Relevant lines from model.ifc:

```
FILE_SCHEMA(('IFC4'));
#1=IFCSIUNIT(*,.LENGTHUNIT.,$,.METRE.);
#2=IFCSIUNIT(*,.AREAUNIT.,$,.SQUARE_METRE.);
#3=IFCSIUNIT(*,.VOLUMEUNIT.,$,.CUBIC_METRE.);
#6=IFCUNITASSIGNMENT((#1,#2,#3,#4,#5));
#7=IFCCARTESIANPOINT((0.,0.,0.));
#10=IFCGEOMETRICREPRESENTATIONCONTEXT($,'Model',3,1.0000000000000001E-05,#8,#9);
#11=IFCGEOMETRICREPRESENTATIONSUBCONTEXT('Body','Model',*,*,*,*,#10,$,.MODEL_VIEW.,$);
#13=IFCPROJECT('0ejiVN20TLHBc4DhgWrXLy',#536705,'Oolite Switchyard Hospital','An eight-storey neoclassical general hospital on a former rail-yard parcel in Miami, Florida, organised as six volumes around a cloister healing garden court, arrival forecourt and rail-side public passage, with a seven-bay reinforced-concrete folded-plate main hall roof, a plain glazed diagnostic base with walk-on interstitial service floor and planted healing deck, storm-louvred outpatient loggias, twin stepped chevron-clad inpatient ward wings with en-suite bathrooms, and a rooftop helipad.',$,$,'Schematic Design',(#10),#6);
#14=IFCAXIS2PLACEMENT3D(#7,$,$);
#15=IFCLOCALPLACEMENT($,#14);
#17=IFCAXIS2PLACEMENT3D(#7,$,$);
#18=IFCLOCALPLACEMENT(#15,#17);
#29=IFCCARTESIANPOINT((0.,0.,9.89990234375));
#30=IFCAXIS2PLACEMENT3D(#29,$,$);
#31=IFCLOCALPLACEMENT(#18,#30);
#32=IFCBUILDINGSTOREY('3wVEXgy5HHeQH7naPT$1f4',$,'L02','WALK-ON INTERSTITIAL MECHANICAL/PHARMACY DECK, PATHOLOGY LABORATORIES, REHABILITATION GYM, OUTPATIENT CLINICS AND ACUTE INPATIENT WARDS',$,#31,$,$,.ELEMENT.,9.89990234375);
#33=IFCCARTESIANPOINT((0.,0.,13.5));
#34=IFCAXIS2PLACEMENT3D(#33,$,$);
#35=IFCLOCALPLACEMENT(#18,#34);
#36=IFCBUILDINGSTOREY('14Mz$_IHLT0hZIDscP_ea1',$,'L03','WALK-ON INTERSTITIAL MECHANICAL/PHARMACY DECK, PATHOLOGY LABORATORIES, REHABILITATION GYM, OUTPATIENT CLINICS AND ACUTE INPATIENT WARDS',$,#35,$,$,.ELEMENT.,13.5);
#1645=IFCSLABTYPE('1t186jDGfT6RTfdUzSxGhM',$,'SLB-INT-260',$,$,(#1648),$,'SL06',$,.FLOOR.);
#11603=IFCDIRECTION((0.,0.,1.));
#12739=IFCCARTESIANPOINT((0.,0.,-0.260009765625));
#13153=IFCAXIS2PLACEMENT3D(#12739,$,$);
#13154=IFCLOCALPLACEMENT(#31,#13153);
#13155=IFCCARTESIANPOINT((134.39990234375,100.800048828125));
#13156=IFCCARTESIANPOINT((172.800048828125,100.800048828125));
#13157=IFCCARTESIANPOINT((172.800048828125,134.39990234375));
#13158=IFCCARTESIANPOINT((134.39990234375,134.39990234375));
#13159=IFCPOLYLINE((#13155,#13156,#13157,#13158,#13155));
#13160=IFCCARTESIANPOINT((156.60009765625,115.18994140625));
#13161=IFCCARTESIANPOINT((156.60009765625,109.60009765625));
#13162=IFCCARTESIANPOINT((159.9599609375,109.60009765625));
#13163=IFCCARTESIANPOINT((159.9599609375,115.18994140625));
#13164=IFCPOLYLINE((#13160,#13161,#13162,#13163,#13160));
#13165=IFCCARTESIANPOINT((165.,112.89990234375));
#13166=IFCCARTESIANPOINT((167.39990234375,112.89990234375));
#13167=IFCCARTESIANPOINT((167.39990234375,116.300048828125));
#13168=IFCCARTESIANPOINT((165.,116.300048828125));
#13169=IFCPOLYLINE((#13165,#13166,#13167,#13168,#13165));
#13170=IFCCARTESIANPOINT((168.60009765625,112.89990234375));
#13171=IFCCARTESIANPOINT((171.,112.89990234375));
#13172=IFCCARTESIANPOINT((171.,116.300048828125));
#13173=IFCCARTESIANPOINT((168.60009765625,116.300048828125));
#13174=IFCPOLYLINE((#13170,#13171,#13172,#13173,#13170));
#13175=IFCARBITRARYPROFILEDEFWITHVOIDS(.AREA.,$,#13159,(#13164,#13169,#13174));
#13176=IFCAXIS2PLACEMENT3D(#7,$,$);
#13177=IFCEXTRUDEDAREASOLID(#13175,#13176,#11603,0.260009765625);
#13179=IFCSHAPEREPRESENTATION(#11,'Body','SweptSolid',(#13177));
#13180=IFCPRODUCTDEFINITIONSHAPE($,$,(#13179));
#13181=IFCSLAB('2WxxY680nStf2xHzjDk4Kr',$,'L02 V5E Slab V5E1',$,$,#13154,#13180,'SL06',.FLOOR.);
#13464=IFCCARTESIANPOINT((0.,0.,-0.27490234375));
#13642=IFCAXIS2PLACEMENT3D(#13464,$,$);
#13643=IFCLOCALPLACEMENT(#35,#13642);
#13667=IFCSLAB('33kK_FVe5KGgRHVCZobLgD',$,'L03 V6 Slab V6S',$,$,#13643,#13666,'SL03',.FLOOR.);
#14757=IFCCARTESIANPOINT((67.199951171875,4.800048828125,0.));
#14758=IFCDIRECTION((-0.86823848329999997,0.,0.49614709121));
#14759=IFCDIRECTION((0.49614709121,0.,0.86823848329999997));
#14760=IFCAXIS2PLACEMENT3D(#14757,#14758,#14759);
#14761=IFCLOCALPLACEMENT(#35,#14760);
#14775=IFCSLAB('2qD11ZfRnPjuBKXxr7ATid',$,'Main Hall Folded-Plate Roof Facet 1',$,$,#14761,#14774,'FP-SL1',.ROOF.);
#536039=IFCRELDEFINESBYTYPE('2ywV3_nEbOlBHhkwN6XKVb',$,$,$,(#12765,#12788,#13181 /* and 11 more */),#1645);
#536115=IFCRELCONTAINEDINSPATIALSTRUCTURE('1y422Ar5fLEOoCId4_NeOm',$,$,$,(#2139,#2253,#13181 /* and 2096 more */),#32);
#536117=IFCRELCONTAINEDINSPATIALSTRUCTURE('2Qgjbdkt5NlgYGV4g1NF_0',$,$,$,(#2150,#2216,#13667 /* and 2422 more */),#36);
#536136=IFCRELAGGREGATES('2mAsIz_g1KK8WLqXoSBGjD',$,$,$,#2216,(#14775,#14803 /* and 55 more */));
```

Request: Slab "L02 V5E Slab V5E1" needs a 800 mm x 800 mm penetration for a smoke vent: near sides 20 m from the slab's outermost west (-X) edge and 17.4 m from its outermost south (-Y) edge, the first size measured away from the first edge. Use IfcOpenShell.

```python
import numpy as np
import ifcopenshell
import ifcopenshell.api.feature
import ifcopenshell.api.geometry
import ifcopenshell.api.root
import ifcopenshell.geom
import ifcopenshell.util.placement
import ifcopenshell.util.representation
import ifcopenshell.util.shape
import ifcopenshell.util.unit

model = ifcopenshell.open("model.ifc")
unit_scale = ifcopenshell.util.unit.calculate_unit_scale(model)
settings = ifcopenshell.geom.settings()


def volume(element):
    """Net volume in cubic metres, openings subtracted."""
    shape = ifcopenshell.geom.create_shape(settings, element)
    return ifcopenshell.util.shape.get_volume(shape.geometry)


slab = model.by_guid("2WxxY680nStf2xHzjDk4Kr")
before = volume(slab)

# Extent in the slab's own axes, in metres. The edges named are its -X and -Y sides.
slab_shape = ifcopenshell.geom.create_shape(settings, slab)
vertices = ifcopenshell.util.shape.get_vertices(slab_shape.geometry)
x_min, y_min, bottom = vertices.min(axis=0)
top = vertices[:, 2].max()

opening = ifcopenshell.api.root.create_entity(model, ifc_class="IfcOpeningElement", name="Smoke vent opening", predefined_type="OPENING")
context = ifcopenshell.util.representation.get_context(model, "Model", "Body", "MODEL_VIEW")
width, depth = 0.8, 0.8
outline = [(0.0, 0.0), (width, 0.0), (width, depth), (0.0, depth), (0.0, 0.0)]
# Overshoot both faces by 50 mm so the cut is clean.
shape = ifcopenshell.api.geometry.add_slab_representation(
    model, context=context, depth=top - bottom + 0.1, polyline=outline
)
ifcopenshell.api.geometry.assign_representation(model, product=opening, representation=shape)

matrix = ifcopenshell.util.placement.get_local_placement(slab.ObjectPlacement)
matrix[:, 3] = matrix @ np.append(np.array([x_min + 20, y_min + 17.4, bottom - 0.05]) / unit_scale, 1.0)
ifcopenshell.api.geometry.edit_object_placement(model, product=opening, matrix=matrix, is_si=False)
ifcopenshell.api.feature.add_feature(model, feature=opening, element=slab)

after = volume(slab)

print(f"slab volume {before:.3f} -> {after:.3f} m3")

model.write("model_updated.ifc")
```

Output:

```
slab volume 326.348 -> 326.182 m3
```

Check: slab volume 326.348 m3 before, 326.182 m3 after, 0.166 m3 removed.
